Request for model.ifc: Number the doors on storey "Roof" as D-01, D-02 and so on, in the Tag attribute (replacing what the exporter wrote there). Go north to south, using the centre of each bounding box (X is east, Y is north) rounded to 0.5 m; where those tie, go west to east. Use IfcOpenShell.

First a look at what the model holds.

```python
import ifcopenshell
import ifcopenshell.util.element
import ifcopenshell.util.placement

model = ifcopenshell.open("model.ifc")
print(model.schema)
storey = next(s for s in model.by_type("IfcBuildingStorey") if s.Name == "Roof")
doors = [e for e in ifcopenshell.util.element.get_decomposition(storey) if e.is_a("IfcDoor")]
for e in sorted(doors, key=lambda e: e.id()):
    origin = ifcopenshell.util.placement.get_local_placement(e.ObjectPlacement)[:3, 3]
    print(e.id(), e.Tag, e.Name, origin.round(2) + 0.0, sep=" | ")
```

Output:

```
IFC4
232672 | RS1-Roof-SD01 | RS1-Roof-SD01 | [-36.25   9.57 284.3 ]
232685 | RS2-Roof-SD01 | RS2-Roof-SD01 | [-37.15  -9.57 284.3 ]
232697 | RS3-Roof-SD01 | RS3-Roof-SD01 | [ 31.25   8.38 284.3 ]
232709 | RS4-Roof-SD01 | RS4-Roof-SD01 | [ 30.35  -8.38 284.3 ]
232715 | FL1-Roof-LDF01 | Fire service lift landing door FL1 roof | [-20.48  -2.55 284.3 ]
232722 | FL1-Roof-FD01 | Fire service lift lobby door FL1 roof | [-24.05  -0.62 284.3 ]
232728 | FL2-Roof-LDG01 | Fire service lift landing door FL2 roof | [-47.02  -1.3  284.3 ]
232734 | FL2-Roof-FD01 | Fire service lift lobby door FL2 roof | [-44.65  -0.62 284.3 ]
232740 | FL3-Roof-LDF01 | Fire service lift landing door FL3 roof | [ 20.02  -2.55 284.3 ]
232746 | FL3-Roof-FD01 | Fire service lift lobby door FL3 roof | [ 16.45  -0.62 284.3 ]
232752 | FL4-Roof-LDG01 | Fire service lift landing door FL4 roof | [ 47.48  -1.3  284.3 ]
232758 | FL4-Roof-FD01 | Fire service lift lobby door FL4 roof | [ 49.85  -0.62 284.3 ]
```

```python
import ifcopenshell
import ifcopenshell.geom
import ifcopenshell.util.element
import ifcopenshell.util.shape

model = ifcopenshell.open("model.ifc")
settings = ifcopenshell.geom.settings()
settings.set("use-world-coords", True)


def centre(element):
    shape = ifcopenshell.geom.create_shape(settings, element)
    return ifcopenshell.util.shape.get_bbox_centroid(shape.geometry)


storey = next(s for s in model.by_type("IfcBuildingStorey") if s.Name == "Roof")
doors = [e for e in ifcopenshell.util.element.get_decomposition(storey) if e.is_a("IfcDoor")]

# Insertion points can sit at a corner or the storey origin, so sort by the geometry (in metres).
centres = {e: centre(e) for e in doors}
doors.sort(key=lambda e: (-round(centres[e][1] / 0.5), centres[e][0]))

for i, e in enumerate(doors, start=1):
    number = f"D-{i:02d}"
    e.Tag = number
    print(e.id(), number)

model.write("model_v2.ifc")
```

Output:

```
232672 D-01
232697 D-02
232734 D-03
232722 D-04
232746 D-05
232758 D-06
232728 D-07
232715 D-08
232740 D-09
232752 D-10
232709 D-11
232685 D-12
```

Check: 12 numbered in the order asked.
